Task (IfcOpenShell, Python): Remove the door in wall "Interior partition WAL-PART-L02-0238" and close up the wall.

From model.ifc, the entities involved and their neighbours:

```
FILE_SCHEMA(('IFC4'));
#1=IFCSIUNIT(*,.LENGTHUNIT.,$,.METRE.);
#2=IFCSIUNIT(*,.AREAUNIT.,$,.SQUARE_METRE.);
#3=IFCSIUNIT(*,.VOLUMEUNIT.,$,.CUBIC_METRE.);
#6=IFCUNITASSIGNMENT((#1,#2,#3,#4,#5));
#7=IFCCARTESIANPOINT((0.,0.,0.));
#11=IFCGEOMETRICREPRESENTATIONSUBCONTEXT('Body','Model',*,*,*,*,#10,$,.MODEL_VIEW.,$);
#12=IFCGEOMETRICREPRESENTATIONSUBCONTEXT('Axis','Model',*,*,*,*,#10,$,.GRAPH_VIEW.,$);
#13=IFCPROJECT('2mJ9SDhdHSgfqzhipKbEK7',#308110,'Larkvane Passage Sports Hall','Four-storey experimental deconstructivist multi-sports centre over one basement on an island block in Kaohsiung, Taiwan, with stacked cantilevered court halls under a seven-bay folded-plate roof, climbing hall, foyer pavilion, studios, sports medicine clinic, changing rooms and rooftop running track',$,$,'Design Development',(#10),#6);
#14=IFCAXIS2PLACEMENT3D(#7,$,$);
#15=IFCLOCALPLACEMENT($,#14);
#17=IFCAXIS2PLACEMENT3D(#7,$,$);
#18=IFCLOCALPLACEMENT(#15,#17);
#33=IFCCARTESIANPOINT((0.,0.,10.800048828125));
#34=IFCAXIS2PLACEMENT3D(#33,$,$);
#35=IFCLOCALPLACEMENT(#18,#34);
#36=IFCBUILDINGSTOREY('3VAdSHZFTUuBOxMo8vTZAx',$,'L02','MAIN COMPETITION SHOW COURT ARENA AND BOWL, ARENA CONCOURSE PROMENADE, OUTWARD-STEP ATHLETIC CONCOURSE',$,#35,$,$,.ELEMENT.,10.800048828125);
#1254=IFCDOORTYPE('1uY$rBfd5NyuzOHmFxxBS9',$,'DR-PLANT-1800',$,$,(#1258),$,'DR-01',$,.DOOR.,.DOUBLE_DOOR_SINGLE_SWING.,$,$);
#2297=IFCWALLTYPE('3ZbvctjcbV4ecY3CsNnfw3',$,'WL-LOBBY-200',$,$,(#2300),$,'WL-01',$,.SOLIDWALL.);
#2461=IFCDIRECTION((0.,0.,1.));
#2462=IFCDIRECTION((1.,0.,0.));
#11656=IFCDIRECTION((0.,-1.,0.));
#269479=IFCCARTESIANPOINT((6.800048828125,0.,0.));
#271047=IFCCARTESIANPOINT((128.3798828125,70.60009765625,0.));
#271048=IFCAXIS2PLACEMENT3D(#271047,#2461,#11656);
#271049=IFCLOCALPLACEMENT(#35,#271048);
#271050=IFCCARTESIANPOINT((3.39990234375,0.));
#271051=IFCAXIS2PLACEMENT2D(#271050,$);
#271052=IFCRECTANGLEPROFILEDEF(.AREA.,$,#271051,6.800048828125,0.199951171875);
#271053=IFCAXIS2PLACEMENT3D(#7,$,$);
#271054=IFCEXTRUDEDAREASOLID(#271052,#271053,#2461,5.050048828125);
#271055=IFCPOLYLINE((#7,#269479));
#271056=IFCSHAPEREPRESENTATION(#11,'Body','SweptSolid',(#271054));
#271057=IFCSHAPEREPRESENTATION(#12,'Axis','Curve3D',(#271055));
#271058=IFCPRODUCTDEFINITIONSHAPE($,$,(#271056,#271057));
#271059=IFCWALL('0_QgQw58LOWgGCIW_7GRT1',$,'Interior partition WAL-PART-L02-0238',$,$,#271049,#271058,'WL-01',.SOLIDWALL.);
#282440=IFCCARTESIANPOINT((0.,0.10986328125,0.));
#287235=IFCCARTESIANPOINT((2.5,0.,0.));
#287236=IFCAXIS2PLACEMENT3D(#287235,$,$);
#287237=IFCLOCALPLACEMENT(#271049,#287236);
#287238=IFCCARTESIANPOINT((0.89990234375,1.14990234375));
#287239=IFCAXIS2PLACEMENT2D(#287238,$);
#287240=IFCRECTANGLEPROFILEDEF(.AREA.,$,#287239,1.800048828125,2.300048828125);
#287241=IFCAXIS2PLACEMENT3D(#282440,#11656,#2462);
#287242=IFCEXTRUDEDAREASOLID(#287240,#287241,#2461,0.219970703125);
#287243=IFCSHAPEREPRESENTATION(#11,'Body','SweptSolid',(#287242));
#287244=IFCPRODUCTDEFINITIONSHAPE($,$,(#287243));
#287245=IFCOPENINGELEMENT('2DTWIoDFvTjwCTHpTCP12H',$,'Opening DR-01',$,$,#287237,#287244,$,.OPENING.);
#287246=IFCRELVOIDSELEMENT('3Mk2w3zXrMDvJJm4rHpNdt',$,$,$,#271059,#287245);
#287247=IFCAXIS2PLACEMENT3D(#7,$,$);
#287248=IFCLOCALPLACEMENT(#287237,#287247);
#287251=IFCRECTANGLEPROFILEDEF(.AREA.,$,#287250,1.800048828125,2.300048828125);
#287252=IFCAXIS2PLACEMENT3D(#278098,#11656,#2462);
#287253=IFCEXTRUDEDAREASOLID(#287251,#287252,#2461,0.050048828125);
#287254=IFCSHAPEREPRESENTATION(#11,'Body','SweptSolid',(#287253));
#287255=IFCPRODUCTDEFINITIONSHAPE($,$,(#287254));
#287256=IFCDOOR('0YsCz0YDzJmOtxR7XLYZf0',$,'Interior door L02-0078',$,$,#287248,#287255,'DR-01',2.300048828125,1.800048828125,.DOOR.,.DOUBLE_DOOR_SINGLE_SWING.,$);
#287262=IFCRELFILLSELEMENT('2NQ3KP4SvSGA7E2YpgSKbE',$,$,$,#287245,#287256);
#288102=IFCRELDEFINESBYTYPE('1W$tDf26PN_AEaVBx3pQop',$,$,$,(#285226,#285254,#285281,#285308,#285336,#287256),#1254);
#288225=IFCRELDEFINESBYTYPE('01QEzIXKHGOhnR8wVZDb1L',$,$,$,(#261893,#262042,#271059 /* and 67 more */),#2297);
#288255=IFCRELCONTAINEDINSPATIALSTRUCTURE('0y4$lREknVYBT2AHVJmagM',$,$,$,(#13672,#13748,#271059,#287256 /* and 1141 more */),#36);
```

```python
import ifcopenshell
import ifcopenshell.api.feature
import ifcopenshell.api.root
import ifcopenshell.geom
import ifcopenshell.util.shape

model = ifcopenshell.open("model.ifc")
settings = ifcopenshell.geom.settings()


def volume(element):
    """Net volume in cubic metres, openings subtracted."""
    shape = ifcopenshell.geom.create_shape(settings, element)
    return ifcopenshell.util.shape.get_volume(shape.geometry)


door = model.by_guid("0YsCz0YDzJmOtxR7XLYZf0")
opening = door.FillsVoids[0].RelatingOpeningElement
wall = opening.VoidsElements[0].RelatingBuildingElement
before = volume(wall)

ifcopenshell.api.root.remove_product(model, product=door)
ifcopenshell.api.feature.remove_feature(model, feature=opening)

after = volume(wall)

print(f"wall volume {before:.3f} -> {after:.3f} m3")

model.write("model_rev.ifc")
```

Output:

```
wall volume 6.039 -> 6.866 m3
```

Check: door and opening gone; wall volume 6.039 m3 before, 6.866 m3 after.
